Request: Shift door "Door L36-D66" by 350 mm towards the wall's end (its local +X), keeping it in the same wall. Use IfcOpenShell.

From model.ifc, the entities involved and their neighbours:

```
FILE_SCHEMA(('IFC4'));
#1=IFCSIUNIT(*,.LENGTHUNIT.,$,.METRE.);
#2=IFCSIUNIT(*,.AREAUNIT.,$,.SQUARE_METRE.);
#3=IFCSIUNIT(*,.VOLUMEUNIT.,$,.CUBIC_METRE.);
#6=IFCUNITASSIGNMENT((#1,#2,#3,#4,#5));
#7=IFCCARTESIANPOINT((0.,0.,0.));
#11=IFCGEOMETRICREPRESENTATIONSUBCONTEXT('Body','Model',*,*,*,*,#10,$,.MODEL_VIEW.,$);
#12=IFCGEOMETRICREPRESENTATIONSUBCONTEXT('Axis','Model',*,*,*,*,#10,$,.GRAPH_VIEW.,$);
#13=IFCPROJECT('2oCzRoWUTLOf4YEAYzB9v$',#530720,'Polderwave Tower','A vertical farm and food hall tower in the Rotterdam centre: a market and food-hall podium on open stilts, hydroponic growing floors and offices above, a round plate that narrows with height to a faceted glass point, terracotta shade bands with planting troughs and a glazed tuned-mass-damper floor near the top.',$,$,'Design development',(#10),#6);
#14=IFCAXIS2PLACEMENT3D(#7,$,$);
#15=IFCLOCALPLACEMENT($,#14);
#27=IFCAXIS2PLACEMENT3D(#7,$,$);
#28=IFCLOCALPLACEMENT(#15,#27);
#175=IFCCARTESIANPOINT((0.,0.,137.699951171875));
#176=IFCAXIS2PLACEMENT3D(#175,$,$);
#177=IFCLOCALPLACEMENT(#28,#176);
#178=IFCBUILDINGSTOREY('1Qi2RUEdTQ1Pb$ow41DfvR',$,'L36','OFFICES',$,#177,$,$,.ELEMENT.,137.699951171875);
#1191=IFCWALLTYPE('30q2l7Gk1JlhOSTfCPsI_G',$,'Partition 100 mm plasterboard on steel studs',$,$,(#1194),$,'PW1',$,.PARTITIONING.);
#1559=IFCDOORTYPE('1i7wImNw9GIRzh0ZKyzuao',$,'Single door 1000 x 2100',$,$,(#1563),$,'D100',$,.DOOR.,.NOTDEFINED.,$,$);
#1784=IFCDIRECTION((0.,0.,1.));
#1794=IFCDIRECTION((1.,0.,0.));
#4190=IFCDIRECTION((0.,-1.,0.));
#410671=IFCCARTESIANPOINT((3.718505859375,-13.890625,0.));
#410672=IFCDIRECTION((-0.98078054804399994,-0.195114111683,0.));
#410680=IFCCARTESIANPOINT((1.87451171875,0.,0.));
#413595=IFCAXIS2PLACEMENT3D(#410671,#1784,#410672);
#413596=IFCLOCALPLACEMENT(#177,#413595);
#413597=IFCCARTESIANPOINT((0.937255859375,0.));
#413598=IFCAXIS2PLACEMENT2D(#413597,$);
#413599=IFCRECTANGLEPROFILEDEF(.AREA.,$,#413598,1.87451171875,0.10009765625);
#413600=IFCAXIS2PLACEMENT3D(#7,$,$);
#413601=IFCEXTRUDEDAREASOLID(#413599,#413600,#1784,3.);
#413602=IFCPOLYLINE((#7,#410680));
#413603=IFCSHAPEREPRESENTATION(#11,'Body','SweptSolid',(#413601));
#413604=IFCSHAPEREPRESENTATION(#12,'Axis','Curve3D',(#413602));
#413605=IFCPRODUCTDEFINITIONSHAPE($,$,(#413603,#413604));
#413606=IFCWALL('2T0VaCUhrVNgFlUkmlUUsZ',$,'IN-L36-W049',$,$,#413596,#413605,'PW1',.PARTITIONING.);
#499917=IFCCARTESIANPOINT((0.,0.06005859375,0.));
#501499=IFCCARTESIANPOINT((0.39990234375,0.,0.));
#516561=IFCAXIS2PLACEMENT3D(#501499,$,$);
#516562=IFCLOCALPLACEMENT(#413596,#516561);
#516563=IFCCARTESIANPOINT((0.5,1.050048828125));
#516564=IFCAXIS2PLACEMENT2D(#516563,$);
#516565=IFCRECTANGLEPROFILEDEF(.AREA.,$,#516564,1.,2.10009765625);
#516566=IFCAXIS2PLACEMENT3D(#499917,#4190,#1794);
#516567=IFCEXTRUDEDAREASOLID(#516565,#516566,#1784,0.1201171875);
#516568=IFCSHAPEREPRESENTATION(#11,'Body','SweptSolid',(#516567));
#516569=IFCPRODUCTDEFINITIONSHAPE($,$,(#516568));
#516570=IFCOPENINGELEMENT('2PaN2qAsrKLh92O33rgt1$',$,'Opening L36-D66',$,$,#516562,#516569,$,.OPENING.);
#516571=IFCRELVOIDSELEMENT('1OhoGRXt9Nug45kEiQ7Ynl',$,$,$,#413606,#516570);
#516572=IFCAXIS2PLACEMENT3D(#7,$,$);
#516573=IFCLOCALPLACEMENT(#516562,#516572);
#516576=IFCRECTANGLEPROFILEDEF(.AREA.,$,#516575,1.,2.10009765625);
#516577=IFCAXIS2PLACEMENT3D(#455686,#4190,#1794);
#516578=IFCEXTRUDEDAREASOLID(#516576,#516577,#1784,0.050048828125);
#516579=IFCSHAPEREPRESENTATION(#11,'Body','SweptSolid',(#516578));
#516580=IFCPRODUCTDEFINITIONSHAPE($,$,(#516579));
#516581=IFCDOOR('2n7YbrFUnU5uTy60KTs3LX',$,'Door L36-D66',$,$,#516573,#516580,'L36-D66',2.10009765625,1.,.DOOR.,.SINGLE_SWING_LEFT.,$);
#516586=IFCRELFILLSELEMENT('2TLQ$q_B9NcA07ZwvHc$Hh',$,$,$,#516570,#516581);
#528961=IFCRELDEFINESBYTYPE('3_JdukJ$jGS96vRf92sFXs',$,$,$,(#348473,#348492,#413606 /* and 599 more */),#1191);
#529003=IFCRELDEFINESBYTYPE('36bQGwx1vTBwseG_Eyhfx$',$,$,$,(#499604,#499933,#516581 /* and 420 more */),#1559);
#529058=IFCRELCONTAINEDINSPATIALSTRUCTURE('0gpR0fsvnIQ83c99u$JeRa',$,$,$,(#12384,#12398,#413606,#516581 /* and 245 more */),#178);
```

```python
import ifcopenshell
import ifcopenshell.api.geometry
import ifcopenshell.util.placement
import ifcopenshell.util.unit

model = ifcopenshell.open("model.ifc")
unit_scale = ifcopenshell.util.unit.calculate_unit_scale(model)

door = model.by_guid("2n7YbrFUnU5uTy60KTs3LX")
opening = door.FillsVoids[0].RelatingOpeningElement
wall = opening.VoidsElements[0].RelatingBuildingElement

wall_matrix = ifcopenshell.util.placement.get_local_placement(wall.ObjectPlacement)
shift = wall_matrix[:3, 0] * 0.35 / unit_scale
before = ifcopenshell.util.placement.get_local_placement(door.ObjectPlacement)[:3, 3].copy()

# The door is placed relative to its opening, so it follows when the opening moves.
matrix = ifcopenshell.util.placement.get_local_placement(opening.ObjectPlacement)
matrix[:3, 3] += shift
ifcopenshell.api.geometry.edit_object_placement(
    model, product=opening, matrix=matrix, is_si=False, should_transform_children=True
)

after = ifcopenshell.util.placement.get_local_placement(door.ObjectPlacement)[:3, 3]
print("door moved by", (after - before).round(3) + 0.0)

model.write("model_v2.ifc")
```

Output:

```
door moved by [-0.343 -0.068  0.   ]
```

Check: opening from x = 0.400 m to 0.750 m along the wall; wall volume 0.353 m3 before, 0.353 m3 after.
